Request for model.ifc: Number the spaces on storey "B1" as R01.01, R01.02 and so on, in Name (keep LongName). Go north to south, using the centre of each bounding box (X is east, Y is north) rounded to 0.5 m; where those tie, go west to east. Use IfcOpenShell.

First a look at what the model holds.

```python
import ifcopenshell
import ifcopenshell.util.element
import ifcopenshell.util.placement

model = ifcopenshell.open("model.ifc")
print(model.schema)
storey = next(s for s in model.by_type("IfcBuildingStorey") if s.Name == "B1")
spaces = [e for e in ifcopenshell.util.element.get_decomposition(storey) if e.is_a("IfcSpace")]
for e in sorted(spaces, key=lambda e: e.id()):
    origin = ifcopenshell.util.placement.get_local_placement(e.ObjectPlacement)[:3, 3]
    print(e.id(), e.Name, e.LongName, origin.round(2) + 0.0, sep=" | ")
```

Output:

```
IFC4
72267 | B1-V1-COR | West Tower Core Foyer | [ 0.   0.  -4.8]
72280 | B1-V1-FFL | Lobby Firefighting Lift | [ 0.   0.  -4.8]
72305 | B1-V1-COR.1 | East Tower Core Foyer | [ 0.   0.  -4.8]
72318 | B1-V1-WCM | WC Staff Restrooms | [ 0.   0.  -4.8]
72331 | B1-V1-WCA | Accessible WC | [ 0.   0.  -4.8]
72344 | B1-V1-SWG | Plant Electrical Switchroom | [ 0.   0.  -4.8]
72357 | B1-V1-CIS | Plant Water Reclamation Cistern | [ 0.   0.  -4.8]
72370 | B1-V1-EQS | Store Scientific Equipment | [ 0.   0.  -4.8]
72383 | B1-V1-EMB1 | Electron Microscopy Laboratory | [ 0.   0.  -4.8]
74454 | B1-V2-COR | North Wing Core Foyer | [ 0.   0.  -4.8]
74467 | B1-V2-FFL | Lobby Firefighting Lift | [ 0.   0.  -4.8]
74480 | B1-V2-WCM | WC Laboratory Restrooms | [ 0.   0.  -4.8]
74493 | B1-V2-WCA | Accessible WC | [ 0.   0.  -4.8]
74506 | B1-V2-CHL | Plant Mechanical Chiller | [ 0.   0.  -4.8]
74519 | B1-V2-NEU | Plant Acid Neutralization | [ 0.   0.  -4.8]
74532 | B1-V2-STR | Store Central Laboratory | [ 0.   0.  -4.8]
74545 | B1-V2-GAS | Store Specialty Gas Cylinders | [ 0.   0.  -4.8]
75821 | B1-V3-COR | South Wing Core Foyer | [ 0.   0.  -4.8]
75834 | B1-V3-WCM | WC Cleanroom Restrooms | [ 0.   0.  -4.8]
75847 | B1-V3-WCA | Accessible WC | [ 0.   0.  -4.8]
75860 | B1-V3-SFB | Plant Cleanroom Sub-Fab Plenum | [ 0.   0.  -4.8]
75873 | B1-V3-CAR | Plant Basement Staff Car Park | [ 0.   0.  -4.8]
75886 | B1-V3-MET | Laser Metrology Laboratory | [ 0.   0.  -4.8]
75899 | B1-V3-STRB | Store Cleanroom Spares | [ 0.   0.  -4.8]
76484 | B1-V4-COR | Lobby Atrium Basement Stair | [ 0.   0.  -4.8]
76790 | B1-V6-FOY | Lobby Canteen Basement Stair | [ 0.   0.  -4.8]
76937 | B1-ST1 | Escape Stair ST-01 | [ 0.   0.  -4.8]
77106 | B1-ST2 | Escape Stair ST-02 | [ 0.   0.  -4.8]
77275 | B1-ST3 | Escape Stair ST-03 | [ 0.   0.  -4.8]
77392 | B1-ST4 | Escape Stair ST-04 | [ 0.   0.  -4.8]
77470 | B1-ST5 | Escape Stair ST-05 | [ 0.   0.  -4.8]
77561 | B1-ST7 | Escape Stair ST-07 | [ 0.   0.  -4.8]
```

```python
import ifcopenshell
import ifcopenshell.geom
import ifcopenshell.util.element
import ifcopenshell.util.shape

model = ifcopenshell.open("model.ifc")
settings = ifcopenshell.geom.settings()
settings.set("use-world-coords", True)


def centre(element):
    shape = ifcopenshell.geom.create_shape(settings, element)
    return ifcopenshell.util.shape.get_bbox_centroid(shape.geometry)


storey = next(s for s in model.by_type("IfcBuildingStorey") if s.Name == "B1")
spaces = [e for e in ifcopenshell.util.element.get_decomposition(storey) if e.is_a("IfcSpace")]

# Insertion points can sit at a corner or the storey origin, so sort by the geometry (in metres).
centres = {e: centre(e) for e in spaces}
spaces.sort(key=lambda e: (-round(centres[e][1] / 0.5), centres[e][0]))

for i, e in enumerate(spaces, start=1):
    number = f"R01.{i:02d}"
    e.Name = number
    print(e.id(), number)

model.write("model_edited.ifc")
```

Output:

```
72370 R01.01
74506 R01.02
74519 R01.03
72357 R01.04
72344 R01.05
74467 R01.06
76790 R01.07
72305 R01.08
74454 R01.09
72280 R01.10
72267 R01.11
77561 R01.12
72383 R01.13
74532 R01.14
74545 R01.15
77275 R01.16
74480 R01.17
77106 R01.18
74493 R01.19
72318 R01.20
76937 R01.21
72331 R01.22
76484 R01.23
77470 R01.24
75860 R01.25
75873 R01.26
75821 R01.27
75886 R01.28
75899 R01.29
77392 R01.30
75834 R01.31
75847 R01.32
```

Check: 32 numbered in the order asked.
